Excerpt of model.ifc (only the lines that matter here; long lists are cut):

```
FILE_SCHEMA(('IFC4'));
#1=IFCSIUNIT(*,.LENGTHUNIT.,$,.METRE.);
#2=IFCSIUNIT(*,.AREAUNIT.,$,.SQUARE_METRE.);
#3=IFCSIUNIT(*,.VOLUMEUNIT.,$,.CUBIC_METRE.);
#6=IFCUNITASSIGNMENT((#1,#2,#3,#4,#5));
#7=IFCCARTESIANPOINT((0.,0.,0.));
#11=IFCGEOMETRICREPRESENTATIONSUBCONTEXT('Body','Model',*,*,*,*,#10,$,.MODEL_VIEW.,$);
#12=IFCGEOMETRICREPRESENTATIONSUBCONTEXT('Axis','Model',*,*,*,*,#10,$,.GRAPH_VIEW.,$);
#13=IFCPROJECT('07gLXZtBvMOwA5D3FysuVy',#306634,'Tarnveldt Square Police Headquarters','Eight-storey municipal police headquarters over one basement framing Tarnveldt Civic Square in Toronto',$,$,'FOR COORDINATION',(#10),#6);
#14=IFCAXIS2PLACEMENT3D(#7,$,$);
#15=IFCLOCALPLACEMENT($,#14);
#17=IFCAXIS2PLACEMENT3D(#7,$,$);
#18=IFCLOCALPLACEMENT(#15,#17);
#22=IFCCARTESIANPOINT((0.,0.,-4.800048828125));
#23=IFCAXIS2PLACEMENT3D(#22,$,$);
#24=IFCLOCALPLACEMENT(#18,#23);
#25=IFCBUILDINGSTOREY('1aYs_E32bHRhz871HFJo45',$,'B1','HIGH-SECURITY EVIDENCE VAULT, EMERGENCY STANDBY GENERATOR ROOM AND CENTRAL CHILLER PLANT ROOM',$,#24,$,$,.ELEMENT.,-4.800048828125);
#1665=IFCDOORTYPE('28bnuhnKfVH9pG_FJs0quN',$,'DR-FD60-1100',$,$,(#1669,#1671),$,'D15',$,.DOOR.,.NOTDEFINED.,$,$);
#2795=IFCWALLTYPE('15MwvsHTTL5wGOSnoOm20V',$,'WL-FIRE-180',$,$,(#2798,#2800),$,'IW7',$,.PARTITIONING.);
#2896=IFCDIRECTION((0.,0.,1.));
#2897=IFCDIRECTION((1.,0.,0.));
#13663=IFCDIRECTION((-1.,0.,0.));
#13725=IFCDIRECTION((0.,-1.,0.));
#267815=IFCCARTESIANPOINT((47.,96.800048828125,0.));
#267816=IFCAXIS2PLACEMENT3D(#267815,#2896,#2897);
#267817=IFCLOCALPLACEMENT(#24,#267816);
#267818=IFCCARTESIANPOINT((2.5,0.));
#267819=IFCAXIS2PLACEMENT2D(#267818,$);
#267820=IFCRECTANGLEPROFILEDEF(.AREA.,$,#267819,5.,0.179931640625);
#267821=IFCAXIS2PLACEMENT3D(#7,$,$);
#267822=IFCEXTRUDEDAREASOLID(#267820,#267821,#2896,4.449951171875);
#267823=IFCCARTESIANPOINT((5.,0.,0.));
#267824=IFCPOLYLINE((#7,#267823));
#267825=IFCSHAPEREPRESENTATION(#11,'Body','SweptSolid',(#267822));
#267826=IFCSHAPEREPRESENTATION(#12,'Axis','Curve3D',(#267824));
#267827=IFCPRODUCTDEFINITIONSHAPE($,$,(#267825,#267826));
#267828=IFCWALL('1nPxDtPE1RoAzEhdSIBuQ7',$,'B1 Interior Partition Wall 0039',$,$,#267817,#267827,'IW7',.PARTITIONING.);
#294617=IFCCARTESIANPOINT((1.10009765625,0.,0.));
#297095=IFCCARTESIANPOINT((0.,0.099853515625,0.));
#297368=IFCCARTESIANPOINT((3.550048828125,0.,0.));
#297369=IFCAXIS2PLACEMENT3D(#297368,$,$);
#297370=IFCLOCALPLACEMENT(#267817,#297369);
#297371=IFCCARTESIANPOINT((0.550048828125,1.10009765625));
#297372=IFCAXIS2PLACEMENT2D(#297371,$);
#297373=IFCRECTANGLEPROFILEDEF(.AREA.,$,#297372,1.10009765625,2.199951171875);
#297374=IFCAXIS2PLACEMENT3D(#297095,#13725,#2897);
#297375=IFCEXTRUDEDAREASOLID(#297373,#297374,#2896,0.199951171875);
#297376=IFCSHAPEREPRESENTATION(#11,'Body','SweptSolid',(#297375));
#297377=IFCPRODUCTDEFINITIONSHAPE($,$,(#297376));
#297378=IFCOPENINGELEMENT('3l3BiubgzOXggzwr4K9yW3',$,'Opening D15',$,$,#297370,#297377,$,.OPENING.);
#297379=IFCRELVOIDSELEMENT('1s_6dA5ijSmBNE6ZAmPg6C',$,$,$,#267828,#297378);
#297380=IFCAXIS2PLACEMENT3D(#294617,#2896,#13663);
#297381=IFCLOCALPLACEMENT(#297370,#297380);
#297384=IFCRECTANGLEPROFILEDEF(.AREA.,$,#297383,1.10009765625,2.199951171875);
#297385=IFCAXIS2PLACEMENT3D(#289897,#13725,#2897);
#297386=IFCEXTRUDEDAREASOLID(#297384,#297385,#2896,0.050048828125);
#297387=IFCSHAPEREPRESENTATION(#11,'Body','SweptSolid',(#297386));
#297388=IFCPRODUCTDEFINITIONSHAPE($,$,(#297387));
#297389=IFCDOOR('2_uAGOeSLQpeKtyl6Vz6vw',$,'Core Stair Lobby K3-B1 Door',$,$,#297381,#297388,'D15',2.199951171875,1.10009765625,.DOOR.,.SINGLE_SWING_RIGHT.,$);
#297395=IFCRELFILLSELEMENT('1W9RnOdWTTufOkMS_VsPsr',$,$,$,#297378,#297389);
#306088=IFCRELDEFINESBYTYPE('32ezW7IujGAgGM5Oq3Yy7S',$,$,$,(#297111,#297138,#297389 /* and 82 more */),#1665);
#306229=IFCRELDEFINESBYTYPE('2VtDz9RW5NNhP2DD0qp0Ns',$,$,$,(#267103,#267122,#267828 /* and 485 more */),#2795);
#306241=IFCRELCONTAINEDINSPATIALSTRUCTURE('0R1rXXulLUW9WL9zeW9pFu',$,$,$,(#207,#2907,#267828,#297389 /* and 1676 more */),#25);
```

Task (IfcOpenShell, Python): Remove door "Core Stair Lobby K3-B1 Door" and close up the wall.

```python
import ifcopenshell
import ifcopenshell.api.feature
import ifcopenshell.api.root
import ifcopenshell.geom
import ifcopenshell.util.shape

model = ifcopenshell.open("model.ifc")
settings = ifcopenshell.geom.settings()


def volume(element):
    """Net volume in cubic metres, openings subtracted."""
    shape = ifcopenshell.geom.create_shape(settings, element)
    return ifcopenshell.util.shape.get_volume(shape.geometry)


door = model.by_guid("2_uAGOeSLQpeKtyl6Vz6vw")
opening = door.FillsVoids[0].RelatingOpeningElement
wall = opening.VoidsElements[0].RelatingBuildingElement
before = volume(wall)

ifcopenshell.api.root.remove_product(model, product=door)
ifcopenshell.api.feature.remove_feature(model, feature=opening)

after = volume(wall)

print(f"wall volume {before:.3f} -> {after:.3f} m3")

model.write("model_rev.ifc")
```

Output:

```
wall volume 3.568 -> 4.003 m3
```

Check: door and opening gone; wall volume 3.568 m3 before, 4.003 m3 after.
